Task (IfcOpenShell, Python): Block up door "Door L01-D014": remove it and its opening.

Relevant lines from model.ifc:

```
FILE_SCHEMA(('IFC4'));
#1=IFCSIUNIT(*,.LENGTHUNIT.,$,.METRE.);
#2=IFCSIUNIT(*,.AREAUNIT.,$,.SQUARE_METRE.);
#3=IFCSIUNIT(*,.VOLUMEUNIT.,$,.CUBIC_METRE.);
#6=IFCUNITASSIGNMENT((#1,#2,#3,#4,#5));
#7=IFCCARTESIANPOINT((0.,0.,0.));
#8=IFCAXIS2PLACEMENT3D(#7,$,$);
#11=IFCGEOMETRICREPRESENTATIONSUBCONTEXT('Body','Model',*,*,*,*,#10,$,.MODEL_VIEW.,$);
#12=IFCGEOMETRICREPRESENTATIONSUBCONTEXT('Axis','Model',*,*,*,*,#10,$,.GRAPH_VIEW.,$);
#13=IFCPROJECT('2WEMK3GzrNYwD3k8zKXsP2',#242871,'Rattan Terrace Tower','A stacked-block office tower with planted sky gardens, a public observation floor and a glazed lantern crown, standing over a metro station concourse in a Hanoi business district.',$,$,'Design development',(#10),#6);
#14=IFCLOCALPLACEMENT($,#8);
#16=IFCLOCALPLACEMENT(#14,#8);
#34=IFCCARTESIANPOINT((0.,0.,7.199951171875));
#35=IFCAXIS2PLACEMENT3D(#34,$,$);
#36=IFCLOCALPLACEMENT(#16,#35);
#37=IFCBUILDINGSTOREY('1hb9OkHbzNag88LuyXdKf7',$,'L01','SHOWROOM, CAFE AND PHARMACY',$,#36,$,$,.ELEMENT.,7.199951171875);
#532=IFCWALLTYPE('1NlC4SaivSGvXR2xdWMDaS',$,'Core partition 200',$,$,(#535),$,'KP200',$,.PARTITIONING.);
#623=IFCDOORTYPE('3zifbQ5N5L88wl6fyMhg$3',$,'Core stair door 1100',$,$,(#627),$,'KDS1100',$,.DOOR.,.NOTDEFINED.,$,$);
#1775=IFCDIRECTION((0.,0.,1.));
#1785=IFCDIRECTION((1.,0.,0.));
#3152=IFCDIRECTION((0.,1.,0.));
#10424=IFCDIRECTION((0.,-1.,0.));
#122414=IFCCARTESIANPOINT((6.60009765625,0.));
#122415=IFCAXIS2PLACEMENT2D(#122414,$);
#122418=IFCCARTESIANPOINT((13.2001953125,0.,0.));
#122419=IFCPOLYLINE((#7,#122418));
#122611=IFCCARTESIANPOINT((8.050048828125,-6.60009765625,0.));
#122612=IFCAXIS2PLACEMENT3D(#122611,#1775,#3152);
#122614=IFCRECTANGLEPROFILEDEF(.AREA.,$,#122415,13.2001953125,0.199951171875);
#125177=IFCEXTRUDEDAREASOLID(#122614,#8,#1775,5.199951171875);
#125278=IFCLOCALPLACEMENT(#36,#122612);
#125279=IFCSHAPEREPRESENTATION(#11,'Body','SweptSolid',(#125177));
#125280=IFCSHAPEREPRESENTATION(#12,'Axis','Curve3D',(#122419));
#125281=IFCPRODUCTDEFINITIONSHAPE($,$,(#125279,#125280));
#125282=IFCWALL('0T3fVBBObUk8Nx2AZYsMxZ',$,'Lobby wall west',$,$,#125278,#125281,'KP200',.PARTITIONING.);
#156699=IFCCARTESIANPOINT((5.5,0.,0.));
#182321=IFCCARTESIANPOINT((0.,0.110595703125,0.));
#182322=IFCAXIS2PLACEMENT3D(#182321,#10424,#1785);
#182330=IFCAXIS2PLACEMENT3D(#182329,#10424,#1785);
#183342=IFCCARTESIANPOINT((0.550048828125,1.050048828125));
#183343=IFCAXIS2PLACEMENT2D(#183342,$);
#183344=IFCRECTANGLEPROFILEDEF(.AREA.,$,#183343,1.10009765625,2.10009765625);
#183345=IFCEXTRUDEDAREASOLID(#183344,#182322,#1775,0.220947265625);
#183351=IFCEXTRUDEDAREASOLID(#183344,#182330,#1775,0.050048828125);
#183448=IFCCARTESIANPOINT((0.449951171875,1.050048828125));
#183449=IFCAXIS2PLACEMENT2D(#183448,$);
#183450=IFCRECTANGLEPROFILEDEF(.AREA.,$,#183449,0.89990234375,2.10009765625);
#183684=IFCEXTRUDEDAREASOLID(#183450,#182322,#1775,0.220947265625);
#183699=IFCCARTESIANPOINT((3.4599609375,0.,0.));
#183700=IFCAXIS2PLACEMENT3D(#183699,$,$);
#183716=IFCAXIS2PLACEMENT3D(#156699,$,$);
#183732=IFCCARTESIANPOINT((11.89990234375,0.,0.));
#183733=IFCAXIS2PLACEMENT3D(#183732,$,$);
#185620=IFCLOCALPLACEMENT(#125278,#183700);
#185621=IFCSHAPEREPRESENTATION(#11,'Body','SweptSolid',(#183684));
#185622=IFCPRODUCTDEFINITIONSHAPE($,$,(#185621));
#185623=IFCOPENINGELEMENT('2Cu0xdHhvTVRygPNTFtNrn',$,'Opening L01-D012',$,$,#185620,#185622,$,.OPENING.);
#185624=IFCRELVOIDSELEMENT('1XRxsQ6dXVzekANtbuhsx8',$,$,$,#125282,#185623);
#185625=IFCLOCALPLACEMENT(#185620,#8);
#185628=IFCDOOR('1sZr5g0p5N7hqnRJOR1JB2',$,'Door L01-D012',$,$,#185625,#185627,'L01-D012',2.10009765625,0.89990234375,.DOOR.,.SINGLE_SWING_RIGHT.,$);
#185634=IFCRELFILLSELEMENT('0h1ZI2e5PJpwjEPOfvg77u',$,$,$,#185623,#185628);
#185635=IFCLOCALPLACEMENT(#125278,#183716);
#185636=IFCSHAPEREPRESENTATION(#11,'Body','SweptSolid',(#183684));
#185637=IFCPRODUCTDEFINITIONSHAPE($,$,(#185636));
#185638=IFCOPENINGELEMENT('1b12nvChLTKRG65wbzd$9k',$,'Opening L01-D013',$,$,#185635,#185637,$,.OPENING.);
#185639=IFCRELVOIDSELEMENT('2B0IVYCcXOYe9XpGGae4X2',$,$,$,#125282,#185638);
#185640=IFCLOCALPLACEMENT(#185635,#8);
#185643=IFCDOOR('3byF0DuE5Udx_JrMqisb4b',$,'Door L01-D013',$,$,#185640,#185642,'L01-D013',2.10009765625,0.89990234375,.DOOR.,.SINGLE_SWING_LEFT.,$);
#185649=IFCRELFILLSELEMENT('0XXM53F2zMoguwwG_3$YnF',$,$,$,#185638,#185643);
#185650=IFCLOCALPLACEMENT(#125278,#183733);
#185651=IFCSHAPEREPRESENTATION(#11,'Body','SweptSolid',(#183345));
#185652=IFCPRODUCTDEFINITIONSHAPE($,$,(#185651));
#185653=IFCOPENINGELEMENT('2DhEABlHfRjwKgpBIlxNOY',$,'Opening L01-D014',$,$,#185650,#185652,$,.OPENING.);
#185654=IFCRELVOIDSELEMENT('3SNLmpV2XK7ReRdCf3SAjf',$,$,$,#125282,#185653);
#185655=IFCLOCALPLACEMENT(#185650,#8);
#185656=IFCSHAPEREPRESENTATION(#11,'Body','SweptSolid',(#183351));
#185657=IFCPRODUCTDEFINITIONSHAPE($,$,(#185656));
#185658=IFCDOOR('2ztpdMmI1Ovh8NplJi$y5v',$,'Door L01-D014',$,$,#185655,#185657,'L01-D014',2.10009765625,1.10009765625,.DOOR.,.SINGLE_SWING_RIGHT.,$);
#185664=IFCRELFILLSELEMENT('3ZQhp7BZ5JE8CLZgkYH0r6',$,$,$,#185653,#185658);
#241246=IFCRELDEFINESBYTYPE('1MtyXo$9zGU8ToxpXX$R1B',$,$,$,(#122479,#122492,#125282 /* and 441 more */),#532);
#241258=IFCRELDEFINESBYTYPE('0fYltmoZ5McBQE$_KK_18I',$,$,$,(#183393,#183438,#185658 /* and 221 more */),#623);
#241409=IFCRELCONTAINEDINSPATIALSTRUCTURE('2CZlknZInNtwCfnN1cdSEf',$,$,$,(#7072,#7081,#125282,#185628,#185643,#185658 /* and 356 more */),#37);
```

```python
import ifcopenshell
import ifcopenshell.api.feature
import ifcopenshell.api.root
import ifcopenshell.geom
import ifcopenshell.util.shape

model = ifcopenshell.open("model.ifc")
settings = ifcopenshell.geom.settings()


def volume(element):
    """Net volume in cubic metres, openings subtracted."""
    shape = ifcopenshell.geom.create_shape(settings, element)
    return ifcopenshell.util.shape.get_volume(shape.geometry)


door = model.by_guid("2ztpdMmI1Ovh8NplJi$y5v")
opening = door.FillsVoids[0].RelatingOpeningElement
wall = opening.VoidsElements[0].RelatingBuildingElement
before = volume(wall)

ifcopenshell.api.root.remove_product(model, product=door)
ifcopenshell.api.feature.remove_feature(model, feature=opening)

after = volume(wall)

print(f"wall volume {before:.3f} -> {after:.3f} m3")

model.write("model-out.ifc")
```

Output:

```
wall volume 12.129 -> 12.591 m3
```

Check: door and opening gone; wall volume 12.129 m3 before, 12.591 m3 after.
